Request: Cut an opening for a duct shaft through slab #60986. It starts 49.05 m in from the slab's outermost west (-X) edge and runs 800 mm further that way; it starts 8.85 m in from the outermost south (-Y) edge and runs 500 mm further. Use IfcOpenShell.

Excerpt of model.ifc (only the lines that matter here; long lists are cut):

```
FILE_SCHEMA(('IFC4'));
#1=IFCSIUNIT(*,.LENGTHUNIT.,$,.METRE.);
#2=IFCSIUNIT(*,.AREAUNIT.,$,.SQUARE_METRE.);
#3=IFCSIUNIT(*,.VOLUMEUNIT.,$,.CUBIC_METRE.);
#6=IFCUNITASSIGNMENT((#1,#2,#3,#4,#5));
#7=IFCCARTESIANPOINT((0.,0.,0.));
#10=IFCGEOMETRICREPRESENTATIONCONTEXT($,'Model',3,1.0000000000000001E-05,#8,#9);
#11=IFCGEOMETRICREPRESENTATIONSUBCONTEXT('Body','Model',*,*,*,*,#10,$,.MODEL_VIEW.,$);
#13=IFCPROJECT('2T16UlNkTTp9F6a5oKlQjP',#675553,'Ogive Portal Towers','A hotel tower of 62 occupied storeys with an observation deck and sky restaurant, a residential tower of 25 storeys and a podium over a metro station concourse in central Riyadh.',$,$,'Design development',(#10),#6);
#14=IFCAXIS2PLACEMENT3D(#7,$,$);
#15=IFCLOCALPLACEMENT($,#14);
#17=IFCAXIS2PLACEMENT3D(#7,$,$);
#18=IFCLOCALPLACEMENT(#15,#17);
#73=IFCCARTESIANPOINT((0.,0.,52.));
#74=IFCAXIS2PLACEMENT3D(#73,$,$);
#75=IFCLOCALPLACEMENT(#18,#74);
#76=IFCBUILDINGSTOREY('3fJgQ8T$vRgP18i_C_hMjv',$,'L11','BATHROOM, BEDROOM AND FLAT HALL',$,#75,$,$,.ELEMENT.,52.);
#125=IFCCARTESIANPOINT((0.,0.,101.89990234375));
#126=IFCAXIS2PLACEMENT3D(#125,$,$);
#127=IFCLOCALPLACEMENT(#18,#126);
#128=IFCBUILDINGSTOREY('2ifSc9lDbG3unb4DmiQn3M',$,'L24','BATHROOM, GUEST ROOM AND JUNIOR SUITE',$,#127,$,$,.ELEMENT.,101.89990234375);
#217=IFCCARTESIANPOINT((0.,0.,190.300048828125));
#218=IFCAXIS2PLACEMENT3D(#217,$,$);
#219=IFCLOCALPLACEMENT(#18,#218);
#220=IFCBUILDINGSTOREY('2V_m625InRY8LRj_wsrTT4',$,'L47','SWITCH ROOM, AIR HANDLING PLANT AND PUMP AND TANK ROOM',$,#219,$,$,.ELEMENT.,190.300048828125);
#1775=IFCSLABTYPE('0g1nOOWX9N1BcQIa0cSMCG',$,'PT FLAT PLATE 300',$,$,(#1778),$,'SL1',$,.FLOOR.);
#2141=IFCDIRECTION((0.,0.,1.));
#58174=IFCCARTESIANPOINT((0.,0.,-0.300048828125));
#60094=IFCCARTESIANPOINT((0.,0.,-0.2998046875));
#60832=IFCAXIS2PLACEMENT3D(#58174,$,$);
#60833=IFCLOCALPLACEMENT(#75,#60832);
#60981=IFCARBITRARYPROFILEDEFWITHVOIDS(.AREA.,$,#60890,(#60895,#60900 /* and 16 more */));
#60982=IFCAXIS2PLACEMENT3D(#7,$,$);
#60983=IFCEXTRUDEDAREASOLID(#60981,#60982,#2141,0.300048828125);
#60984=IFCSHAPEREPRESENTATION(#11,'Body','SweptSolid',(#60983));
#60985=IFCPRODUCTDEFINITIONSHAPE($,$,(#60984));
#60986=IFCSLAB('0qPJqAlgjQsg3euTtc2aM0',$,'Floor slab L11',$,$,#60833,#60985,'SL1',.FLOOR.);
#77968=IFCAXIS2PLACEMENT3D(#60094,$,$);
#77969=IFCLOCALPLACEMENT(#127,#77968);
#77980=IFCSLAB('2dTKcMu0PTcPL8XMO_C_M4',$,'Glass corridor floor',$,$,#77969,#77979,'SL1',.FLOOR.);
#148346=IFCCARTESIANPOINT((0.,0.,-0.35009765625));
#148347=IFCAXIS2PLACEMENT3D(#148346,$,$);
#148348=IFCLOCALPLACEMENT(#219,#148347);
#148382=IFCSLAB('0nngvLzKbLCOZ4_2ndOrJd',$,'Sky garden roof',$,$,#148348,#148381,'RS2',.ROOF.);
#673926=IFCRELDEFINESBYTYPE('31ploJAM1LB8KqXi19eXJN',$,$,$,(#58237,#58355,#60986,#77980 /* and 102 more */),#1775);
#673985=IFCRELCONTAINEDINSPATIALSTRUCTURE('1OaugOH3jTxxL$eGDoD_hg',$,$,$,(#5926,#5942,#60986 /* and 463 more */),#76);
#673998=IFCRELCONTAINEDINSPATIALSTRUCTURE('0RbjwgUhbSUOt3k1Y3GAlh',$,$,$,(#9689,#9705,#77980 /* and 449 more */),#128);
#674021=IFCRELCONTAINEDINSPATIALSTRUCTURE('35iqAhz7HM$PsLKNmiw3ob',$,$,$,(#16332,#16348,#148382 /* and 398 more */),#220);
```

```python
import numpy as np
import ifcopenshell
import ifcopenshell.api.feature
import ifcopenshell.api.geometry
import ifcopenshell.api.root
import ifcopenshell.geom
import ifcopenshell.util.placement
import ifcopenshell.util.representation
import ifcopenshell.util.shape
import ifcopenshell.util.unit

model = ifcopenshell.open("model.ifc")
unit_scale = ifcopenshell.util.unit.calculate_unit_scale(model)
settings = ifcopenshell.geom.settings()


def volume(element):
    """Net volume in cubic metres, openings subtracted."""
    shape = ifcopenshell.geom.create_shape(settings, element)
    return ifcopenshell.util.shape.get_volume(shape.geometry)


slab = model.by_guid("0qPJqAlgjQsg3euTtc2aM0")
before = volume(slab)

# Extent in the slab's own axes, in metres. The edges named are its -X and -Y sides.
slab_shape = ifcopenshell.geom.create_shape(settings, slab)
vertices = ifcopenshell.util.shape.get_vertices(slab_shape.geometry)
x_min, y_min, bottom = vertices.min(axis=0)
top = vertices[:, 2].max()

opening = ifcopenshell.api.root.create_entity(model, ifc_class="IfcOpeningElement", name="Duct shaft opening", predefined_type="OPENING")
context = ifcopenshell.util.representation.get_context(model, "Model", "Body", "MODEL_VIEW")
width, depth = 0.8, 0.5
outline = [(0.0, 0.0), (width, 0.0), (width, depth), (0.0, depth), (0.0, 0.0)]
# Overshoot both faces by 50 mm so the cut is clean.
shape = ifcopenshell.api.geometry.add_slab_representation(
    model, context=context, depth=top - bottom + 0.1, polyline=outline
)
ifcopenshell.api.geometry.assign_representation(model, product=opening, representation=shape)

matrix = ifcopenshell.util.placement.get_local_placement(slab.ObjectPlacement)
matrix[:, 3] = matrix @ np.append(np.array([x_min + 49.05, y_min + 8.85, bottom - 0.05]) / unit_scale, 1.0)
ifcopenshell.api.geometry.edit_object_placement(model, product=opening, matrix=matrix, is_si=False)
ifcopenshell.api.feature.add_feature(model, feature=opening, element=slab)

after = volume(slab)

print(f"slab volume {before:.3f} -> {after:.3f} m3")

model.write("model_updated.ifc")
```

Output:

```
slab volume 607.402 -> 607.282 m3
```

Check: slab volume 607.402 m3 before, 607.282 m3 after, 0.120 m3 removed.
